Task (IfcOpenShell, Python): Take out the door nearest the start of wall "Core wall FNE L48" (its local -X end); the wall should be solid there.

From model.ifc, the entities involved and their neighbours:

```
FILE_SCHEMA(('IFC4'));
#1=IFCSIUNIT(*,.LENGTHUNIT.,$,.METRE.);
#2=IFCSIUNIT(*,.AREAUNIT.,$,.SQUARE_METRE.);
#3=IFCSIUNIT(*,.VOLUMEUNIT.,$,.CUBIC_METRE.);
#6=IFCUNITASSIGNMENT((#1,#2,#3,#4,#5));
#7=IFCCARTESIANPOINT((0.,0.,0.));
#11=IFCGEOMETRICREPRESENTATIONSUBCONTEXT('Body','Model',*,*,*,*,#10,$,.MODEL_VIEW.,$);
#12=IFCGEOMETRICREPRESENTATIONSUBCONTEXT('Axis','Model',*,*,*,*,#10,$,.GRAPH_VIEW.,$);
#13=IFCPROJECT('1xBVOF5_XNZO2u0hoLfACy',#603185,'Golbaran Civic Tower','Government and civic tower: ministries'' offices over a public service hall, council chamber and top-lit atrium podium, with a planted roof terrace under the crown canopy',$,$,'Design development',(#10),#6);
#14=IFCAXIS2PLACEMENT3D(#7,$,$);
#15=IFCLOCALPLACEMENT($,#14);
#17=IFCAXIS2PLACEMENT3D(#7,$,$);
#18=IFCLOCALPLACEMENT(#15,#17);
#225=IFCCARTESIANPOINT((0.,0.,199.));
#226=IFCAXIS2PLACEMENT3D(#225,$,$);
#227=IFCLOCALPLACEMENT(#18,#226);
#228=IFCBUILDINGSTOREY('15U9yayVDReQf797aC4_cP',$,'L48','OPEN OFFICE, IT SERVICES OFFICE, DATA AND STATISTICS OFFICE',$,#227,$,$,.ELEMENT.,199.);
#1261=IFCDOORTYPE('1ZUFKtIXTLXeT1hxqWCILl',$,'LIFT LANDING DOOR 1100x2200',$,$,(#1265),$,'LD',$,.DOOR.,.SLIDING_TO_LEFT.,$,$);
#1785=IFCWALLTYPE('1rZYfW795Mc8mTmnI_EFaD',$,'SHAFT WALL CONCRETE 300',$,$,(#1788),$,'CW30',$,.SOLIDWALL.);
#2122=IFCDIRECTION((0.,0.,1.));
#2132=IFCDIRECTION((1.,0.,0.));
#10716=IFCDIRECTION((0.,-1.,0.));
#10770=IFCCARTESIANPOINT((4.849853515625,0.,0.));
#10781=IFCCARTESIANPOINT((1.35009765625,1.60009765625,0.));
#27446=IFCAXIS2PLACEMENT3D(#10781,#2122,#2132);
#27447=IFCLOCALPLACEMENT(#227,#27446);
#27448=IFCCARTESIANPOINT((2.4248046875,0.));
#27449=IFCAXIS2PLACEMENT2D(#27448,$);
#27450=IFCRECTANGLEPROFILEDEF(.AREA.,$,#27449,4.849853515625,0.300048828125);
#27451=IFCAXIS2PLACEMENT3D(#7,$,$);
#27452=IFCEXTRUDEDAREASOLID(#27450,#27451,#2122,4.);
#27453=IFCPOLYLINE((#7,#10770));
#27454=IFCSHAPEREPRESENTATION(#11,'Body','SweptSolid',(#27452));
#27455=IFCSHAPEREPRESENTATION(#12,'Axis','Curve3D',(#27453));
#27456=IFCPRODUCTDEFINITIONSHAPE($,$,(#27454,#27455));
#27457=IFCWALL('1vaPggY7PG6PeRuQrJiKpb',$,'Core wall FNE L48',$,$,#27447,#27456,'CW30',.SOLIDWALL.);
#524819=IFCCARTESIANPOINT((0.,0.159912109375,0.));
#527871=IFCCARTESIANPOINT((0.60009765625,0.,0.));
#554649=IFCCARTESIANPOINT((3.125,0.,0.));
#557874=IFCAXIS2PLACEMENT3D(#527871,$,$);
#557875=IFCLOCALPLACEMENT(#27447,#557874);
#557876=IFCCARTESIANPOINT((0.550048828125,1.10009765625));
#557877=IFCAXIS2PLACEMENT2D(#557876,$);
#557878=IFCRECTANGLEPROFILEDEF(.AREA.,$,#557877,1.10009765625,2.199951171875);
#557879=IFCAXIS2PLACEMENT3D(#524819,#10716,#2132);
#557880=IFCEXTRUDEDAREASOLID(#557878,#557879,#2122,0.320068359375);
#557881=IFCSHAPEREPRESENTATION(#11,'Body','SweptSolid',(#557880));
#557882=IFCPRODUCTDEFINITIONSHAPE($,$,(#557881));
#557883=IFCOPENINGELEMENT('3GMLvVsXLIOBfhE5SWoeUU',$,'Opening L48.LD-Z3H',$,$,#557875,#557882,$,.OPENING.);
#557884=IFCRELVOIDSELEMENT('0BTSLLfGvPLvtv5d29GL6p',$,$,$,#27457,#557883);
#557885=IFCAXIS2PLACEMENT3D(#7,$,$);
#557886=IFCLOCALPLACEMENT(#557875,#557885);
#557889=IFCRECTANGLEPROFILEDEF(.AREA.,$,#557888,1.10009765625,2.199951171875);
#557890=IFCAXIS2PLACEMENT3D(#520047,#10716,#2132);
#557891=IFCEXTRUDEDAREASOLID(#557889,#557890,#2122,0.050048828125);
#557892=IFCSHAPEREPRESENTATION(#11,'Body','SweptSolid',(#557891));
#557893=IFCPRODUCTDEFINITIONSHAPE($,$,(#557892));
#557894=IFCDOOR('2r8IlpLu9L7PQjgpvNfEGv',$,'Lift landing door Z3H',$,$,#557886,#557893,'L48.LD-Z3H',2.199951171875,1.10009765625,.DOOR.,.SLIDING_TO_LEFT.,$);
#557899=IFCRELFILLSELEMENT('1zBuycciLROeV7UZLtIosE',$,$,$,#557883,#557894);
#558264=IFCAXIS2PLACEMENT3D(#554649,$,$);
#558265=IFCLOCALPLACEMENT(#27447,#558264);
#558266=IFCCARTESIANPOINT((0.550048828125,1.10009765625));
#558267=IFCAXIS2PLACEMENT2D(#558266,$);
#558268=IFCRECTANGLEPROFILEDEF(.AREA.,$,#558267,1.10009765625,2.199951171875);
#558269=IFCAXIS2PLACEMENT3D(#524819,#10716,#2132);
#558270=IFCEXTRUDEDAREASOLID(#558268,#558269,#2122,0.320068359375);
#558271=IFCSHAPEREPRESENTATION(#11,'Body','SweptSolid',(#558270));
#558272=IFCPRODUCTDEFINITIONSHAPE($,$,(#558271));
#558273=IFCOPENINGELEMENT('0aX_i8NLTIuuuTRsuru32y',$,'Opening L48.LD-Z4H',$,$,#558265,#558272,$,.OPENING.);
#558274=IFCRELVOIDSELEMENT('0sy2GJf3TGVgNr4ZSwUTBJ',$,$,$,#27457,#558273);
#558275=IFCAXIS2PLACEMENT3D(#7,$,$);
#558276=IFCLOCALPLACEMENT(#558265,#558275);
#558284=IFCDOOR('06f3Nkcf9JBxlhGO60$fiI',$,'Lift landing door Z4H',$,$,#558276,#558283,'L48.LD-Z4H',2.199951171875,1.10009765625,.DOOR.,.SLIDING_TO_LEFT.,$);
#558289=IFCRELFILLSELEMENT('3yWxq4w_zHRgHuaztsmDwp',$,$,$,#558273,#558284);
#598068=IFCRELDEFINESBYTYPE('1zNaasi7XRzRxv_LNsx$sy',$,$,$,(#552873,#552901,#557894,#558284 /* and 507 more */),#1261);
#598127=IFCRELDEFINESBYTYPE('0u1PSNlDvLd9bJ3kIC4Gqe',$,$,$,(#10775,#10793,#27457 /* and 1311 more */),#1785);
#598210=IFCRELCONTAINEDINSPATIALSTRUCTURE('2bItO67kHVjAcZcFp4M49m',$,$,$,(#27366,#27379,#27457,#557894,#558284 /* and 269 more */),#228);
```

```python
import ifcopenshell
import ifcopenshell.api.feature
import ifcopenshell.api.root
import ifcopenshell.geom
import ifcopenshell.util.shape

model = ifcopenshell.open("model.ifc")
settings = ifcopenshell.geom.settings()


def volume(element):
    """Net volume in cubic metres, openings subtracted."""
    shape = ifcopenshell.geom.create_shape(settings, element)
    return ifcopenshell.util.shape.get_volume(shape.geometry)


door = model.by_guid("2r8IlpLu9L7PQjgpvNfEGv")
opening = door.FillsVoids[0].RelatingOpeningElement
wall = opening.VoidsElements[0].RelatingBuildingElement
before = volume(wall)

ifcopenshell.api.root.remove_product(model, product=door)
ifcopenshell.api.feature.remove_feature(model, feature=opening)

after = volume(wall)

print(f"wall volume {before:.3f} -> {after:.3f} m3")

model.write("model-out.ifc")
```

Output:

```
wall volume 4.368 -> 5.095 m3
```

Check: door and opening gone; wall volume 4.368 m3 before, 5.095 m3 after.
